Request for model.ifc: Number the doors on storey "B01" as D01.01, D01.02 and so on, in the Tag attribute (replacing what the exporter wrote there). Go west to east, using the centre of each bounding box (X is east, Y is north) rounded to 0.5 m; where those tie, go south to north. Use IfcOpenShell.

First a look at what the model holds.

```python
import ifcopenshell
import ifcopenshell.util.element
import ifcopenshell.util.placement

model = ifcopenshell.open("model.ifc")
print(model.schema)
storey = next(s for s in model.by_type("IfcBuildingStorey") if s.Name == "B01")
doors = [e for e in ifcopenshell.util.element.get_decomposition(storey) if e.is_a("IfcDoor")]
for e in sorted(doors, key=lambda e: e.id()):
    origin = ifcopenshell.util.placement.get_local_placement(e.ObjectPlacement)[:3, 3]
    print(e.id(), e.Tag, e.Name, origin.round(2) + 0.0, sep=" | ")
```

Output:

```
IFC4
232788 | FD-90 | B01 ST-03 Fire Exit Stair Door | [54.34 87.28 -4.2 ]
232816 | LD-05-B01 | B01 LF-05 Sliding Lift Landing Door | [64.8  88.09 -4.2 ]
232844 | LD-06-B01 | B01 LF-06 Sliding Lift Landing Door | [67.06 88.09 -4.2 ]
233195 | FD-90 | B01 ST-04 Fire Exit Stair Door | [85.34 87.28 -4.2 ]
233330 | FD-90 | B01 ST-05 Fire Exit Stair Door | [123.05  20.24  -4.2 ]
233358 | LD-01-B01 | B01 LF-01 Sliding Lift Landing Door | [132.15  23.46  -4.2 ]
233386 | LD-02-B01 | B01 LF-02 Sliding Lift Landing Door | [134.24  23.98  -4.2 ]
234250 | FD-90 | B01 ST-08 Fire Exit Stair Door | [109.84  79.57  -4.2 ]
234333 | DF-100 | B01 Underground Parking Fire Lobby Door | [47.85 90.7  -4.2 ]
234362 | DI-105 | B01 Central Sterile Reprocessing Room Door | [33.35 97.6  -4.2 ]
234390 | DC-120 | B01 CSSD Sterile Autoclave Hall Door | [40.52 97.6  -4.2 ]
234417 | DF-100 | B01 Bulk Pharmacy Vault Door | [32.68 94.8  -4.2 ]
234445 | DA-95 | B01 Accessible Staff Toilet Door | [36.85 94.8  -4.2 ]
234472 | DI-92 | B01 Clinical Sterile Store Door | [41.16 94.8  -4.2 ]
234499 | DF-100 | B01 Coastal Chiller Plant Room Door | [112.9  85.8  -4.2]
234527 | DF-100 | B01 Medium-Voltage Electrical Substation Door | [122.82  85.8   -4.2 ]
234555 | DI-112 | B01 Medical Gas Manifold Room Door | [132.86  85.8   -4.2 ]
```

```python
import ifcopenshell
import ifcopenshell.geom
import ifcopenshell.util.element
import ifcopenshell.util.shape

model = ifcopenshell.open("model.ifc")
settings = ifcopenshell.geom.settings()
settings.set("use-world-coords", True)


def centre(element):
    shape = ifcopenshell.geom.create_shape(settings, element)
    return ifcopenshell.util.shape.get_bbox_centroid(shape.geometry)


storey = next(s for s in model.by_type("IfcBuildingStorey") if s.Name == "B01")
doors = [e for e in ifcopenshell.util.element.get_decomposition(storey) if e.is_a("IfcDoor")]

# Insertion points can sit at a corner or the storey origin, so sort by the geometry (in metres).
centres = {e: centre(e) for e in doors}
doors.sort(key=lambda e: (round(centres[e][0] / 0.5), centres[e][1]))

for i, e in enumerate(doors, start=1):
    number = f"D01.{i:02d}"
    e.Tag = number
    print(e.id(), number)

model.write("model_edited.ifc")
```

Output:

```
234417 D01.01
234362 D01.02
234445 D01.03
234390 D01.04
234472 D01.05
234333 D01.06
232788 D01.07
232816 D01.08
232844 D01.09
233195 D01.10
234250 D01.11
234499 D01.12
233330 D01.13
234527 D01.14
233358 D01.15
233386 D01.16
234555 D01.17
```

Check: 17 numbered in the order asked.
